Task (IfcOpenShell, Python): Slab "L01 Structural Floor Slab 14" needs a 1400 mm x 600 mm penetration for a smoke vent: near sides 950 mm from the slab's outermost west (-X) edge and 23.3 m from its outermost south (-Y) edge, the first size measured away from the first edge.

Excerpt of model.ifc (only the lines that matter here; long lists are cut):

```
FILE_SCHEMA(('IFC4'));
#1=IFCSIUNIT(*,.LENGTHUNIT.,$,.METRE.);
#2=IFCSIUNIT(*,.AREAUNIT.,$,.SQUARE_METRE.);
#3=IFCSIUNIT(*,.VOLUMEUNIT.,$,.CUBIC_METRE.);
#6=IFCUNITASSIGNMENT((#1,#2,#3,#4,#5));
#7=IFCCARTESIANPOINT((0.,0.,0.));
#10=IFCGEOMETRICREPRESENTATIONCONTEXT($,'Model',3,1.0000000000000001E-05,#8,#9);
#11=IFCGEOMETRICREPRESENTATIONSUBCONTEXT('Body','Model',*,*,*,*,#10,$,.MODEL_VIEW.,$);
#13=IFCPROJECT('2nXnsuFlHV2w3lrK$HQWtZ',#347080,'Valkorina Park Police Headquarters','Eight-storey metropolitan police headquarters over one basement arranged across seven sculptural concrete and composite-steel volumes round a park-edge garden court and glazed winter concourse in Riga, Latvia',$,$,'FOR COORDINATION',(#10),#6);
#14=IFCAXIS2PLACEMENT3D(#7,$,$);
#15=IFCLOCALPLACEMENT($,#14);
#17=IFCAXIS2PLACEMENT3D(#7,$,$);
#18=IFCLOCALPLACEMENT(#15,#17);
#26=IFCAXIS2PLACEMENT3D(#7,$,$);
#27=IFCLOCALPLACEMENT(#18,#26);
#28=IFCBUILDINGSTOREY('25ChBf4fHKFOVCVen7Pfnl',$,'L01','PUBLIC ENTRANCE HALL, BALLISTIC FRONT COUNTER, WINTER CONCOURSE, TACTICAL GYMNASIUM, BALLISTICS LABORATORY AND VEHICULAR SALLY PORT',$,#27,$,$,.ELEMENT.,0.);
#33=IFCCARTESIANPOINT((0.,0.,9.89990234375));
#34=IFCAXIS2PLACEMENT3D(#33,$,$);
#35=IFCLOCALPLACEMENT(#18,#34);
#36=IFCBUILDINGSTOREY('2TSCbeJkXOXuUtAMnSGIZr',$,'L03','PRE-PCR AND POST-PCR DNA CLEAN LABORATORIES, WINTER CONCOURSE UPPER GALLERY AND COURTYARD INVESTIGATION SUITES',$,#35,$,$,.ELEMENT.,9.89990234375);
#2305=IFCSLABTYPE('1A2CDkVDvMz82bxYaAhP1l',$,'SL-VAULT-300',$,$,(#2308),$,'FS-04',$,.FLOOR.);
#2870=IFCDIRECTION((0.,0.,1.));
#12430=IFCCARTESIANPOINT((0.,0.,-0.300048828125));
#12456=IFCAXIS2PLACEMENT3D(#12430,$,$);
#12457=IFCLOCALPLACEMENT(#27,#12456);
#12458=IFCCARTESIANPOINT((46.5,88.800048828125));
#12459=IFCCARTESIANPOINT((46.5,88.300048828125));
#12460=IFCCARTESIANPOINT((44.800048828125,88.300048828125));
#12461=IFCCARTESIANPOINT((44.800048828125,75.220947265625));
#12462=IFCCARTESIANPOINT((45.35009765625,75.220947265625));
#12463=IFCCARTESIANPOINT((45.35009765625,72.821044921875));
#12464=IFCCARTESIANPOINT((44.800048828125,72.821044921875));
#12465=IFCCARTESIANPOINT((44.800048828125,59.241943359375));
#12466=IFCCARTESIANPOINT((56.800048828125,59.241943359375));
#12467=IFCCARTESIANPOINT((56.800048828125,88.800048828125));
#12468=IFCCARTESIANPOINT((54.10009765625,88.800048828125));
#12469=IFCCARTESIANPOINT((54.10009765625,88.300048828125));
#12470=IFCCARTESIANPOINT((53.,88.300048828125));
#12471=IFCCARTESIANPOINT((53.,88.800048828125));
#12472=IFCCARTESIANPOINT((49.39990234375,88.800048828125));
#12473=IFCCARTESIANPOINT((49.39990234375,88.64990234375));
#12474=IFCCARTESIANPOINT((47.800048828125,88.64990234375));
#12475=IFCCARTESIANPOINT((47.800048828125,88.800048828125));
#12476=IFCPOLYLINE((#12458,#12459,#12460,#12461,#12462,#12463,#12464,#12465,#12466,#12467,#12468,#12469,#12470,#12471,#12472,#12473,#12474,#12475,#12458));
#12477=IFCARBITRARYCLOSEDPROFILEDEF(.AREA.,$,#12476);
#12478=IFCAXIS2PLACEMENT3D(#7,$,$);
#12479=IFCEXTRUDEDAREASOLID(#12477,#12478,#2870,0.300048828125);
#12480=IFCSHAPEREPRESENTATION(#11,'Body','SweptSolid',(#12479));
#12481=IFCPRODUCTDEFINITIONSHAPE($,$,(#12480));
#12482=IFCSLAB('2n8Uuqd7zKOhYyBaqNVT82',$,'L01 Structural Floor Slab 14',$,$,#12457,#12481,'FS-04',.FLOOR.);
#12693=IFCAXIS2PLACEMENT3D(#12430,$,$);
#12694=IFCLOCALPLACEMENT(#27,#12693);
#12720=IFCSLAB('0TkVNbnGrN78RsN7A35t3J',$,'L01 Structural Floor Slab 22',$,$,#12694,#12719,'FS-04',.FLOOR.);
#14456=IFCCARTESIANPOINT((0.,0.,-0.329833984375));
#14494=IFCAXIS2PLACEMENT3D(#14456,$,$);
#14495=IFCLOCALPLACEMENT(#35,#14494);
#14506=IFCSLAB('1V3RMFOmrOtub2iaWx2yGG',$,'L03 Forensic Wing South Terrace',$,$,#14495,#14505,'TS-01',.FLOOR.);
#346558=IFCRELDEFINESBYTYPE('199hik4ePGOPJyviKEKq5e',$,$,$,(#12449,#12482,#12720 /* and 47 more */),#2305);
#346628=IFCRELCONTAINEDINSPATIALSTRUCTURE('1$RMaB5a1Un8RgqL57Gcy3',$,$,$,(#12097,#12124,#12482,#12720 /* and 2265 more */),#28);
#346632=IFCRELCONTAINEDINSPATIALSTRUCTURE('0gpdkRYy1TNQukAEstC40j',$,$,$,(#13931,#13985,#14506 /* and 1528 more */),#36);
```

```python
import numpy as np
import ifcopenshell
import ifcopenshell.api.feature
import ifcopenshell.api.geometry
import ifcopenshell.api.root
import ifcopenshell.geom
import ifcopenshell.util.placement
import ifcopenshell.util.representation
import ifcopenshell.util.shape
import ifcopenshell.util.unit

model = ifcopenshell.open("model.ifc")
unit_scale = ifcopenshell.util.unit.calculate_unit_scale(model)
settings = ifcopenshell.geom.settings()


def volume(element):
    """Net volume in cubic metres, openings subtracted."""
    shape = ifcopenshell.geom.create_shape(settings, element)
    return ifcopenshell.util.shape.get_volume(shape.geometry)


slab = model.by_guid("2n8Uuqd7zKOhYyBaqNVT82")
before = volume(slab)

# Extent in the slab's own axes, in metres. The edges named are its -X and -Y sides.
slab_shape = ifcopenshell.geom.create_shape(settings, slab)
vertices = ifcopenshell.util.shape.get_vertices(slab_shape.geometry)
x_min, y_min, bottom = vertices.min(axis=0)
top = vertices[:, 2].max()

opening = ifcopenshell.api.root.create_entity(model, ifc_class="IfcOpeningElement", name="Smoke vent opening", predefined_type="OPENING")
context = ifcopenshell.util.representation.get_context(model, "Model", "Body", "MODEL_VIEW")
width, depth = 1.4, 0.6
outline = [(0.0, 0.0), (width, 0.0), (width, depth), (0.0, depth), (0.0, 0.0)]
# Overshoot both faces by 50 mm so the cut is clean.
shape = ifcopenshell.api.geometry.add_slab_representation(
    model, context=context, depth=top - bottom + 0.1, polyline=outline
)
ifcopenshell.api.geometry.assign_representation(model, product=opening, representation=shape)

matrix = ifcopenshell.util.placement.get_local_placement(slab.ObjectPlacement)
matrix[:, 3] = matrix @ np.append(np.array([x_min + 0.95, y_min + 23.3, bottom - 0.05]) / unit_scale, 1.0)
ifcopenshell.api.geometry.edit_object_placement(model, product=opening, matrix=matrix, is_si=False)
ifcopenshell.api.feature.add_feature(model, feature=opening, element=slab)

after = volume(slab)

print(f"slab volume {before:.3f} -> {after:.3f} m3")

model.write("model_edited.ifc")
```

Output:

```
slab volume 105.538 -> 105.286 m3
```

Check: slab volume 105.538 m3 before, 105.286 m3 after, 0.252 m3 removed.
